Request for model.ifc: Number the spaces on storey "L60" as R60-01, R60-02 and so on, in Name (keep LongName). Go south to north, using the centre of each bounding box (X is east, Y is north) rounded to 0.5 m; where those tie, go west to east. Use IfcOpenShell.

First a look at what the model holds.

```python
import ifcopenshell
import ifcopenshell.util.element
import ifcopenshell.util.placement

model = ifcopenshell.open("model.ifc")
print(model.schema)
storey = next(s for s in model.by_type("IfcBuildingStorey") if s.Name == "L60")
spaces = [e for e in ifcopenshell.util.element.get_decomposition(storey) if e.is_a("IfcSpace")]
for e in sorted(spaces, key=lambda e: e.id()):
    origin = ifcopenshell.util.placement.get_local_placement(e.ObjectPlacement)[:3, 3]
    print(e.id(), e.Name, e.LongName, origin.round(2) + 0.0, sep=" | ")
```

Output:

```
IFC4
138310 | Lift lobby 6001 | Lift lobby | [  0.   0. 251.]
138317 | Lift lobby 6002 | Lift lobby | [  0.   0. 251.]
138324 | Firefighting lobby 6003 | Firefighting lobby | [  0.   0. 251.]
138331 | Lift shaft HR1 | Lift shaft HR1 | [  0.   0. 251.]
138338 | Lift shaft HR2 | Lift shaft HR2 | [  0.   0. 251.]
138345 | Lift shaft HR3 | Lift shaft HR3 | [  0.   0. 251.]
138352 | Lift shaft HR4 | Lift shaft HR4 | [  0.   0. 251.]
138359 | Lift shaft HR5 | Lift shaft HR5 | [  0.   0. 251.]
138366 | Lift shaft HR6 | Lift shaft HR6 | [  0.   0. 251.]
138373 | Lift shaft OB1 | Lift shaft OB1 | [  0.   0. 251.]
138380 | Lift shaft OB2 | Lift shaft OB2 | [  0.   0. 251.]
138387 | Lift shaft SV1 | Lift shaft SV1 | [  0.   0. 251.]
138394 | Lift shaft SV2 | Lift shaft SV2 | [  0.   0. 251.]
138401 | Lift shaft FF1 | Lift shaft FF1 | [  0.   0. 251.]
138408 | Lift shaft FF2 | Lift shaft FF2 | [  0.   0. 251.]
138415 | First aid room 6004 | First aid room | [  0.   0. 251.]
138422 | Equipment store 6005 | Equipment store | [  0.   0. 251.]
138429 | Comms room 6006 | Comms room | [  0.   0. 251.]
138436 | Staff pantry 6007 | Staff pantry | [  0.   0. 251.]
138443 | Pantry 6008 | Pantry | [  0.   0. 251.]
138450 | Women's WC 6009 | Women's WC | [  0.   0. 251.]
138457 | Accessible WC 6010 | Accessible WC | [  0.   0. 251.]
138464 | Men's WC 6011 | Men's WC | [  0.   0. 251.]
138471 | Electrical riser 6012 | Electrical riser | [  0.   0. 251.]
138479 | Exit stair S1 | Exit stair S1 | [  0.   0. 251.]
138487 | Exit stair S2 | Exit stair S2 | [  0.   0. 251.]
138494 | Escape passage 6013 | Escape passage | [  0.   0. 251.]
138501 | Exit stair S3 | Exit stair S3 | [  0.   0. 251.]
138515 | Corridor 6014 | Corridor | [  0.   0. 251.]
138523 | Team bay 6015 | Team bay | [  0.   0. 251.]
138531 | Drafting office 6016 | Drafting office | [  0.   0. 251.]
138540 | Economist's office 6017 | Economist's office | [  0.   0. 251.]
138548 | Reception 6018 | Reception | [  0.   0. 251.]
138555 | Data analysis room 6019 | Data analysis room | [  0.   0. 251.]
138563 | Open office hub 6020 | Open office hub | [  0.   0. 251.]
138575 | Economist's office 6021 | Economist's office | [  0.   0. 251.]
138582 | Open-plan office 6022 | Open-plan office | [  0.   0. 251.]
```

```python
import ifcopenshell
import ifcopenshell.geom
import ifcopenshell.util.element
import ifcopenshell.util.shape

model = ifcopenshell.open("model.ifc")
settings = ifcopenshell.geom.settings()
settings.set("use-world-coords", True)


def centre(element):
    shape = ifcopenshell.geom.create_shape(settings, element)
    return ifcopenshell.util.shape.get_bbox_centroid(shape.geometry)


storey = next(s for s in model.by_type("IfcBuildingStorey") if s.Name == "L60")
spaces = [e for e in ifcopenshell.util.element.get_decomposition(storey) if e.is_a("IfcSpace")]

# Insertion points can sit at a corner or the storey origin, so sort by the geometry (in metres).
centres = {e: centre(e) for e in spaces}
spaces.sort(key=lambda e: (round(centres[e][1] / 0.5), centres[e][0]))

for i, e in enumerate(spaces, start=1):
    number = f"R60-{i:02d}"
    e.Name = number
    print(e.id(), number)

model.write("model_rev.ifc")
```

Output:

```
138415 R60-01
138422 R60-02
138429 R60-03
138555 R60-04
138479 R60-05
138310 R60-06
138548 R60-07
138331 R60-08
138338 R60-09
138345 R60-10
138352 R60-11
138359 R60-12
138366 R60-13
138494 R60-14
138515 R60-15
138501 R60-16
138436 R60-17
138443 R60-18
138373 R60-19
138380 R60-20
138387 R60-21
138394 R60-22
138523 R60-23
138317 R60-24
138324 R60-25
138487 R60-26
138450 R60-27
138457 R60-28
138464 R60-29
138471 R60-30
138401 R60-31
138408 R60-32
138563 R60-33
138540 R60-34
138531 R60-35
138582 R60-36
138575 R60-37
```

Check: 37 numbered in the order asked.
